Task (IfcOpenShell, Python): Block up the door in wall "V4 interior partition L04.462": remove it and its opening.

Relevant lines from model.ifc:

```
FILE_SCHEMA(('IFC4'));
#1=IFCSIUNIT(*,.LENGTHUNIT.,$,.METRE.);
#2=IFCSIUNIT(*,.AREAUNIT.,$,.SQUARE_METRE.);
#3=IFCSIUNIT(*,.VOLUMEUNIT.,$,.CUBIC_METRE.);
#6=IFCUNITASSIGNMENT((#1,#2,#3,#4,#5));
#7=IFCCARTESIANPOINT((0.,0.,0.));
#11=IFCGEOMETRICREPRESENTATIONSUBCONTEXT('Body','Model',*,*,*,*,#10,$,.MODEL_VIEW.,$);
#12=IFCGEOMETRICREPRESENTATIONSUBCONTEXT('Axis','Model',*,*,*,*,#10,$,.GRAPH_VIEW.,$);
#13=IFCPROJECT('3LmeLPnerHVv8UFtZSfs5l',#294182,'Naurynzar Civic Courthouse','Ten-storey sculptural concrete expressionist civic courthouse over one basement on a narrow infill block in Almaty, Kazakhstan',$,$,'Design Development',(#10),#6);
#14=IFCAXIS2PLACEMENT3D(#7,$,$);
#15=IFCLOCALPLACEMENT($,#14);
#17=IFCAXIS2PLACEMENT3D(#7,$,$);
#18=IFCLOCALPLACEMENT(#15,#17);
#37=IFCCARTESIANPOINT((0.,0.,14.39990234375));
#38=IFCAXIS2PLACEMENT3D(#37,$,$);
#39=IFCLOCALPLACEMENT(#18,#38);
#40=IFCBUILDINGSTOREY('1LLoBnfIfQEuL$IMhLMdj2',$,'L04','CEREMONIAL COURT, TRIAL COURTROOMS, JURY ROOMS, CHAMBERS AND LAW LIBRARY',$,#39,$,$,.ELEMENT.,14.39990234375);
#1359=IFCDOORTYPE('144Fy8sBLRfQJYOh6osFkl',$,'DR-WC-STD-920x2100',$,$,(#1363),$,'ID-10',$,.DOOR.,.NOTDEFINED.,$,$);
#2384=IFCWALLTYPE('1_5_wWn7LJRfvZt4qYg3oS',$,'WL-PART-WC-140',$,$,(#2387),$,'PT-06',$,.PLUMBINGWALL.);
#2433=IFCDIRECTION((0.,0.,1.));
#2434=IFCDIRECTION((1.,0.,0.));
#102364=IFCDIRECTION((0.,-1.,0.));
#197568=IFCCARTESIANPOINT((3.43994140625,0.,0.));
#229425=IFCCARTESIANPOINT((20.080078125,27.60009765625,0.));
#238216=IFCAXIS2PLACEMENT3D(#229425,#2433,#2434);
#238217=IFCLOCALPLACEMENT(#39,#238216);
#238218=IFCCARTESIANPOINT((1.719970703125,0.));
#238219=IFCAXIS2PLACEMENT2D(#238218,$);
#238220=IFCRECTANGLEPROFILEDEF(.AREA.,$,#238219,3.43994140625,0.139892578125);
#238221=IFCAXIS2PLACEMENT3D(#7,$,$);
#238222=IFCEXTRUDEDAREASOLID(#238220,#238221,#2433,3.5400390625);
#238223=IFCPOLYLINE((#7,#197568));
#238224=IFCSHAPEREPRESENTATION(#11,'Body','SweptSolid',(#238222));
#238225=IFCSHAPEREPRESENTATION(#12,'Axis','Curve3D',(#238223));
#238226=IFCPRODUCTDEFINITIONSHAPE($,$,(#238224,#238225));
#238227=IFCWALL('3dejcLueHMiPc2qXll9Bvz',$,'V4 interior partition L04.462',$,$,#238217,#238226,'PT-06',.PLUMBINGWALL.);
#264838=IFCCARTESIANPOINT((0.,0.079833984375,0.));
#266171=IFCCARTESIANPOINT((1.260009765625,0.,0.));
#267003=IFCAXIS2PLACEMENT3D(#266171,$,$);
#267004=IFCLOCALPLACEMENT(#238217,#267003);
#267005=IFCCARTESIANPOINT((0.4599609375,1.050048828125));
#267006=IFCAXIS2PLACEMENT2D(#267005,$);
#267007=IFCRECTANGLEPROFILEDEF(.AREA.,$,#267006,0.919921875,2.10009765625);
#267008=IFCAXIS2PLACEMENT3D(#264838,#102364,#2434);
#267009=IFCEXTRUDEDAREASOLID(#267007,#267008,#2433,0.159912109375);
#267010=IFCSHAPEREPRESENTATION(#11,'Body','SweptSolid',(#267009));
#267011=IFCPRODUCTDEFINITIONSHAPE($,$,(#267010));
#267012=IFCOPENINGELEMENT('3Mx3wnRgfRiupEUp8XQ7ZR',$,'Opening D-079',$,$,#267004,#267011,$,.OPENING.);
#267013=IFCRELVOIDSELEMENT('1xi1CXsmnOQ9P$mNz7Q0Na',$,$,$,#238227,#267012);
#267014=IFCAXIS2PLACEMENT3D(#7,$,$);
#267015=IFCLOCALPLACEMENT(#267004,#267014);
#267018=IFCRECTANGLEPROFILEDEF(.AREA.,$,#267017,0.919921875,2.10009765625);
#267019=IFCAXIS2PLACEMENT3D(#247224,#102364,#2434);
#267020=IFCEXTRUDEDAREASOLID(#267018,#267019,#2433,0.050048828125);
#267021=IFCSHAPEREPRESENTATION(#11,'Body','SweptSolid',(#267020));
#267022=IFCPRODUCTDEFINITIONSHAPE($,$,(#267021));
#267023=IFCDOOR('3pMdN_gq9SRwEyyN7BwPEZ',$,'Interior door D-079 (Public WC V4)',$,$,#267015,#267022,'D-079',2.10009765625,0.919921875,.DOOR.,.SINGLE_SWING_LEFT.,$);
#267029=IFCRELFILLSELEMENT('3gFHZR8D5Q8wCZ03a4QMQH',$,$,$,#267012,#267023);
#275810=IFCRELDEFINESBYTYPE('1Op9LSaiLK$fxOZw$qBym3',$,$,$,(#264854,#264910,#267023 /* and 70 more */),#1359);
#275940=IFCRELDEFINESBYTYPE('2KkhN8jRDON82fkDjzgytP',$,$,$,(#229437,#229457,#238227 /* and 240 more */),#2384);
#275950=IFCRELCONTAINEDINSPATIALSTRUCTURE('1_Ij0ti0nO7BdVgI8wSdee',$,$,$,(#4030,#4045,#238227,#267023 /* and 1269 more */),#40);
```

```python
import ifcopenshell
import ifcopenshell.api.feature
import ifcopenshell.api.root
import ifcopenshell.geom
import ifcopenshell.util.shape

model = ifcopenshell.open("model.ifc")
settings = ifcopenshell.geom.settings()


def volume(element):
    """Net volume in cubic metres, openings subtracted."""
    shape = ifcopenshell.geom.create_shape(settings, element)
    return ifcopenshell.util.shape.get_volume(shape.geometry)


door = model.by_id(267023)
opening = door.FillsVoids[0].RelatingOpeningElement
wall = opening.VoidsElements[0].RelatingBuildingElement
before = volume(wall)

ifcopenshell.api.root.remove_product(model, product=door)
ifcopenshell.api.feature.remove_feature(model, feature=opening)

after = volume(wall)

print(f"wall volume {before:.3f} -> {after:.3f} m3")

model.write("model-out.ifc")
```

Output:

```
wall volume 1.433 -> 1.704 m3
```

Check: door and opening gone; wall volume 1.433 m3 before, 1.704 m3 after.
